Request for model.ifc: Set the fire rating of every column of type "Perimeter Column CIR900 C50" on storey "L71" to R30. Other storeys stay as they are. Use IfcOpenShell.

First a look at what the model holds.

```python
import ifcopenshell
import ifcopenshell.util.element

model = ifcopenshell.open("model.ifc")
print(model.schema)
storey = next(s for s in model.by_type("IfcBuildingStorey") if s.Name == "L71")
columns = [e for e in ifcopenshell.util.element.get_decomposition(storey) if e.is_a("IfcColumn")]
seen = {}
for e in columns:
    element_type = ifcopenshell.util.element.get_type(e)
    key = (element_type.Name if element_type != e and element_type else None, ifcopenshell.util.element.get_pset(e, "Pset_ColumnCommon", "FireRating"))
    seen[key] = seen.get(key, 0) + 1
for (name, value), count in sorted(seen.items(), key=str):
    print(count, "x", name, "|", value)
```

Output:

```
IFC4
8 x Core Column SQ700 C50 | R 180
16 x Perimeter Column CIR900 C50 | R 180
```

```python
import ifcopenshell
import ifcopenshell.api.pset
import ifcopenshell.util.element

model = ifcopenshell.open("model.ifc")

storey = next(s for s in model.by_type("IfcBuildingStorey") if s.Name == "L71")
columns = [e for e in ifcopenshell.util.element.get_decomposition(storey) if e.is_a("IfcColumn")]

count = 0
for e in columns:
    element_type = ifcopenshell.util.element.get_type(e)
    if element_type in (None, e) or element_type.Name != "Perimeter Column CIR900 C50":
        continue
    found = ifcopenshell.util.element.get_pset(e, "Pset_ColumnCommon", should_inherit=False)
    if found:
        pset = model.by_id(found["id"])
        if len(ifcopenshell.util.element.get_elements_by_pset(pset)) > 1:
            pset = ifcopenshell.api.pset.unshare_pset(model, products=[e], pset=pset)[0]
    else:
        pset = ifcopenshell.api.pset.add_pset(model, product=e, name="Pset_ColumnCommon")
    ifcopenshell.api.pset.edit_pset(model, pset=pset, properties={"FireRating": "R30"})
    count += 1

print(count, "columns updated")

model.write("model_edited.ifc")
```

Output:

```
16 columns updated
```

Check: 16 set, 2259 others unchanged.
